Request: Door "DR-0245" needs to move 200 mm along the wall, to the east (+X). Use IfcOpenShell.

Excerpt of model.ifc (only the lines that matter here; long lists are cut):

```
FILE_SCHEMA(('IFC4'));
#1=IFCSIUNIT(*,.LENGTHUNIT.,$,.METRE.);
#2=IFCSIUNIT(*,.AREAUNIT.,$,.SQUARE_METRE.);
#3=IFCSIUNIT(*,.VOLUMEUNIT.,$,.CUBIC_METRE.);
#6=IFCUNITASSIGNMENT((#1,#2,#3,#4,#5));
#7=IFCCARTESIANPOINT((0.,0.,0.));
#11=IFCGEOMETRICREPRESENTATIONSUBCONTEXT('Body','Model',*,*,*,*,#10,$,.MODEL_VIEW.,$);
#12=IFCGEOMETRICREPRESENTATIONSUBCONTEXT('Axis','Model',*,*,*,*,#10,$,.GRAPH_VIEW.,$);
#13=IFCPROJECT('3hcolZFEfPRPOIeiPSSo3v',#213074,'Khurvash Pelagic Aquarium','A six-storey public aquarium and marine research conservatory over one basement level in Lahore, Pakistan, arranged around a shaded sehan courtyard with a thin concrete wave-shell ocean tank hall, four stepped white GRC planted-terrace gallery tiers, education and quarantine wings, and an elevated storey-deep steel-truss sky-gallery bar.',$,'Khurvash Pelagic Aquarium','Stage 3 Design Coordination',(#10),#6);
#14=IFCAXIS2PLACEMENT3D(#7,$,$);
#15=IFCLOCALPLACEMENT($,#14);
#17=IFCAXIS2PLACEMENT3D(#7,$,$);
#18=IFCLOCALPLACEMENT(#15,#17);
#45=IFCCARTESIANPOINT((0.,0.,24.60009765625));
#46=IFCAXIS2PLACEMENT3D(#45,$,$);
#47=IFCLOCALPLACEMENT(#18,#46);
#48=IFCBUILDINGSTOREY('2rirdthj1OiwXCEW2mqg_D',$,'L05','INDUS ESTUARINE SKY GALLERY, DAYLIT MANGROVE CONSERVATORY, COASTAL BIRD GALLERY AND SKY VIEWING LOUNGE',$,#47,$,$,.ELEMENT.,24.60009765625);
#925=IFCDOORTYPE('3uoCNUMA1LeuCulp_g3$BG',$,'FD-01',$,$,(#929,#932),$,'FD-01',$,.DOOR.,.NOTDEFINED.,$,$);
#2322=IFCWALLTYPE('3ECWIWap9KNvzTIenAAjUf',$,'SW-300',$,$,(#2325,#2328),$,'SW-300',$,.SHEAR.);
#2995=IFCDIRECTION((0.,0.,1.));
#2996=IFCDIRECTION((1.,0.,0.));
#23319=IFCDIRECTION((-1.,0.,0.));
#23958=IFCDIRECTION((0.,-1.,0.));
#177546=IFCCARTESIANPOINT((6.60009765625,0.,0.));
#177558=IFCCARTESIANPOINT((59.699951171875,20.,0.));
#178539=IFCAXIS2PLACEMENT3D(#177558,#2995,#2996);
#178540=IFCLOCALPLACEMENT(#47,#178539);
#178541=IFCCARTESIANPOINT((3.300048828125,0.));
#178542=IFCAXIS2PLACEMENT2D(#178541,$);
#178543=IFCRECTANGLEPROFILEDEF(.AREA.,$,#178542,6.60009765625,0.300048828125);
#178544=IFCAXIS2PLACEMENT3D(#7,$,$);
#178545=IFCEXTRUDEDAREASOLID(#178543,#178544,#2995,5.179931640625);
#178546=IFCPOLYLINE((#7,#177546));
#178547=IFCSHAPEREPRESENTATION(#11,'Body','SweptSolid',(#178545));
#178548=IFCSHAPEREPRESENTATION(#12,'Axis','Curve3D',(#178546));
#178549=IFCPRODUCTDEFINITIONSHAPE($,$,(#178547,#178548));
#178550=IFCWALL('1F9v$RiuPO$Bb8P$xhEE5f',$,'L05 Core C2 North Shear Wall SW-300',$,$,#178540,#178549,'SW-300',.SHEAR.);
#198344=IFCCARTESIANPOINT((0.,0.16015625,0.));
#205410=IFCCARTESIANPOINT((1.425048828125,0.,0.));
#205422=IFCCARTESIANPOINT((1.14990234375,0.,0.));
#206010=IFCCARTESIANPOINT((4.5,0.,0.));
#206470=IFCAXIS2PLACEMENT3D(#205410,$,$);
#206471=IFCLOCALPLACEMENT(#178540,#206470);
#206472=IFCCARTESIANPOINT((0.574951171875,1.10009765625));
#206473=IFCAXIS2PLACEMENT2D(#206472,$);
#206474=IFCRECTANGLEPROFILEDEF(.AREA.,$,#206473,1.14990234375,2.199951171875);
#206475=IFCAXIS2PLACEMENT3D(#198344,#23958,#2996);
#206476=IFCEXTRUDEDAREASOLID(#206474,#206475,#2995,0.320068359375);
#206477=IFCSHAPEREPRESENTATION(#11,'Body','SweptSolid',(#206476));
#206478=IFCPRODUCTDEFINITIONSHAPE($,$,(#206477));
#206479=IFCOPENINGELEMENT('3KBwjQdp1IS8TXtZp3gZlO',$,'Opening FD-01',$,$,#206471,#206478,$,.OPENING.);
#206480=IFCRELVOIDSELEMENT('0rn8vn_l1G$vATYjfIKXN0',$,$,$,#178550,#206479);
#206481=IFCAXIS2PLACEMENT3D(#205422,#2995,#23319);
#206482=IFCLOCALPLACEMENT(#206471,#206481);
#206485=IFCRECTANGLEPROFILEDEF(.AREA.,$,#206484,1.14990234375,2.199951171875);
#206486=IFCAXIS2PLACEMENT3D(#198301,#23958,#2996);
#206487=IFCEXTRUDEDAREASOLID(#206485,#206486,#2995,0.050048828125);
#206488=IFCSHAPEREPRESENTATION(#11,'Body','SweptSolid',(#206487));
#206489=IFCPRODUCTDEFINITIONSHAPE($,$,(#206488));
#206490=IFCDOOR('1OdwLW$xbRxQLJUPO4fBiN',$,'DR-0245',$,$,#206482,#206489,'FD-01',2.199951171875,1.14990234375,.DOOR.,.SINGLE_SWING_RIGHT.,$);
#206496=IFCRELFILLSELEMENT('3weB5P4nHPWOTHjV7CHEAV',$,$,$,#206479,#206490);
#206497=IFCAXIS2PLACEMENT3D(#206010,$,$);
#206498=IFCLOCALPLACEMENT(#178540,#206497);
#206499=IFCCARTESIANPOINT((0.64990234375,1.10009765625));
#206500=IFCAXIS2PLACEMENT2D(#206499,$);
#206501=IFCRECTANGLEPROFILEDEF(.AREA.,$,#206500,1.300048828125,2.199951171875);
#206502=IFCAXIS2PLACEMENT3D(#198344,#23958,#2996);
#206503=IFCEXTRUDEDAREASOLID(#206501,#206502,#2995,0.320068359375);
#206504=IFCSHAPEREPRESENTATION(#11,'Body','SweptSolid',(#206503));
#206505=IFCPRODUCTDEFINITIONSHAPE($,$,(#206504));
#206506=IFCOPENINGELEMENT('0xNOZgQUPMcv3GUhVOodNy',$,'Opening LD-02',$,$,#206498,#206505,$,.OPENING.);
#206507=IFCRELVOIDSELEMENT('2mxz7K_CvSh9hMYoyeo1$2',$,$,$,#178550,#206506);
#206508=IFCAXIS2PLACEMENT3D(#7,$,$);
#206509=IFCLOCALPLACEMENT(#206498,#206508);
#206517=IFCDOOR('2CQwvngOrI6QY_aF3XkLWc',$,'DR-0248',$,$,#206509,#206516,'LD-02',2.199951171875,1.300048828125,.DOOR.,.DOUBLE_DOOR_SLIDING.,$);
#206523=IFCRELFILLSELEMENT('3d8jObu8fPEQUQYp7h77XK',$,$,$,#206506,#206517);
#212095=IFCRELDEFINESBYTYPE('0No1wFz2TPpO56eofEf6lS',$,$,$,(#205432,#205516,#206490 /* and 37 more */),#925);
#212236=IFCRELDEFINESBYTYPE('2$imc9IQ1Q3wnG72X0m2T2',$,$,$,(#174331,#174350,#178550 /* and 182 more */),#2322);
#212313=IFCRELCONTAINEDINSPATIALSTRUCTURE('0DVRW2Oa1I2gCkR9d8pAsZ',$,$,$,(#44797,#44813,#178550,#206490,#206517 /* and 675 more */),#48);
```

```python
import ifcopenshell
import ifcopenshell.api.geometry
import ifcopenshell.util.placement

model = ifcopenshell.open("model.ifc")

door = model.by_id(206490)
opening = door.FillsVoids[0].RelatingOpeningElement
wall = opening.VoidsElements[0].RelatingBuildingElement

wall_matrix = ifcopenshell.util.placement.get_local_placement(wall.ObjectPlacement)
shift = wall_matrix[:3, 0] * 0.2
before = ifcopenshell.util.placement.get_local_placement(door.ObjectPlacement)[:3, 3].copy()

# The door is placed relative to its opening, so it follows when the opening moves.
matrix = ifcopenshell.util.placement.get_local_placement(opening.ObjectPlacement)
matrix[:3, 3] += shift
ifcopenshell.api.geometry.edit_object_placement(
    model, product=opening, matrix=matrix, is_si=False, should_transform_children=True
)

after = ifcopenshell.util.placement.get_local_placement(door.ObjectPlacement)[:3, 3]
print("door moved by", (after - before).round(3) + 0.0)

model.write("model_edited.ifc")
```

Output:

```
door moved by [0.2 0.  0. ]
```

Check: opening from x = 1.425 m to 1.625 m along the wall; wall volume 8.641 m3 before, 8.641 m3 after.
